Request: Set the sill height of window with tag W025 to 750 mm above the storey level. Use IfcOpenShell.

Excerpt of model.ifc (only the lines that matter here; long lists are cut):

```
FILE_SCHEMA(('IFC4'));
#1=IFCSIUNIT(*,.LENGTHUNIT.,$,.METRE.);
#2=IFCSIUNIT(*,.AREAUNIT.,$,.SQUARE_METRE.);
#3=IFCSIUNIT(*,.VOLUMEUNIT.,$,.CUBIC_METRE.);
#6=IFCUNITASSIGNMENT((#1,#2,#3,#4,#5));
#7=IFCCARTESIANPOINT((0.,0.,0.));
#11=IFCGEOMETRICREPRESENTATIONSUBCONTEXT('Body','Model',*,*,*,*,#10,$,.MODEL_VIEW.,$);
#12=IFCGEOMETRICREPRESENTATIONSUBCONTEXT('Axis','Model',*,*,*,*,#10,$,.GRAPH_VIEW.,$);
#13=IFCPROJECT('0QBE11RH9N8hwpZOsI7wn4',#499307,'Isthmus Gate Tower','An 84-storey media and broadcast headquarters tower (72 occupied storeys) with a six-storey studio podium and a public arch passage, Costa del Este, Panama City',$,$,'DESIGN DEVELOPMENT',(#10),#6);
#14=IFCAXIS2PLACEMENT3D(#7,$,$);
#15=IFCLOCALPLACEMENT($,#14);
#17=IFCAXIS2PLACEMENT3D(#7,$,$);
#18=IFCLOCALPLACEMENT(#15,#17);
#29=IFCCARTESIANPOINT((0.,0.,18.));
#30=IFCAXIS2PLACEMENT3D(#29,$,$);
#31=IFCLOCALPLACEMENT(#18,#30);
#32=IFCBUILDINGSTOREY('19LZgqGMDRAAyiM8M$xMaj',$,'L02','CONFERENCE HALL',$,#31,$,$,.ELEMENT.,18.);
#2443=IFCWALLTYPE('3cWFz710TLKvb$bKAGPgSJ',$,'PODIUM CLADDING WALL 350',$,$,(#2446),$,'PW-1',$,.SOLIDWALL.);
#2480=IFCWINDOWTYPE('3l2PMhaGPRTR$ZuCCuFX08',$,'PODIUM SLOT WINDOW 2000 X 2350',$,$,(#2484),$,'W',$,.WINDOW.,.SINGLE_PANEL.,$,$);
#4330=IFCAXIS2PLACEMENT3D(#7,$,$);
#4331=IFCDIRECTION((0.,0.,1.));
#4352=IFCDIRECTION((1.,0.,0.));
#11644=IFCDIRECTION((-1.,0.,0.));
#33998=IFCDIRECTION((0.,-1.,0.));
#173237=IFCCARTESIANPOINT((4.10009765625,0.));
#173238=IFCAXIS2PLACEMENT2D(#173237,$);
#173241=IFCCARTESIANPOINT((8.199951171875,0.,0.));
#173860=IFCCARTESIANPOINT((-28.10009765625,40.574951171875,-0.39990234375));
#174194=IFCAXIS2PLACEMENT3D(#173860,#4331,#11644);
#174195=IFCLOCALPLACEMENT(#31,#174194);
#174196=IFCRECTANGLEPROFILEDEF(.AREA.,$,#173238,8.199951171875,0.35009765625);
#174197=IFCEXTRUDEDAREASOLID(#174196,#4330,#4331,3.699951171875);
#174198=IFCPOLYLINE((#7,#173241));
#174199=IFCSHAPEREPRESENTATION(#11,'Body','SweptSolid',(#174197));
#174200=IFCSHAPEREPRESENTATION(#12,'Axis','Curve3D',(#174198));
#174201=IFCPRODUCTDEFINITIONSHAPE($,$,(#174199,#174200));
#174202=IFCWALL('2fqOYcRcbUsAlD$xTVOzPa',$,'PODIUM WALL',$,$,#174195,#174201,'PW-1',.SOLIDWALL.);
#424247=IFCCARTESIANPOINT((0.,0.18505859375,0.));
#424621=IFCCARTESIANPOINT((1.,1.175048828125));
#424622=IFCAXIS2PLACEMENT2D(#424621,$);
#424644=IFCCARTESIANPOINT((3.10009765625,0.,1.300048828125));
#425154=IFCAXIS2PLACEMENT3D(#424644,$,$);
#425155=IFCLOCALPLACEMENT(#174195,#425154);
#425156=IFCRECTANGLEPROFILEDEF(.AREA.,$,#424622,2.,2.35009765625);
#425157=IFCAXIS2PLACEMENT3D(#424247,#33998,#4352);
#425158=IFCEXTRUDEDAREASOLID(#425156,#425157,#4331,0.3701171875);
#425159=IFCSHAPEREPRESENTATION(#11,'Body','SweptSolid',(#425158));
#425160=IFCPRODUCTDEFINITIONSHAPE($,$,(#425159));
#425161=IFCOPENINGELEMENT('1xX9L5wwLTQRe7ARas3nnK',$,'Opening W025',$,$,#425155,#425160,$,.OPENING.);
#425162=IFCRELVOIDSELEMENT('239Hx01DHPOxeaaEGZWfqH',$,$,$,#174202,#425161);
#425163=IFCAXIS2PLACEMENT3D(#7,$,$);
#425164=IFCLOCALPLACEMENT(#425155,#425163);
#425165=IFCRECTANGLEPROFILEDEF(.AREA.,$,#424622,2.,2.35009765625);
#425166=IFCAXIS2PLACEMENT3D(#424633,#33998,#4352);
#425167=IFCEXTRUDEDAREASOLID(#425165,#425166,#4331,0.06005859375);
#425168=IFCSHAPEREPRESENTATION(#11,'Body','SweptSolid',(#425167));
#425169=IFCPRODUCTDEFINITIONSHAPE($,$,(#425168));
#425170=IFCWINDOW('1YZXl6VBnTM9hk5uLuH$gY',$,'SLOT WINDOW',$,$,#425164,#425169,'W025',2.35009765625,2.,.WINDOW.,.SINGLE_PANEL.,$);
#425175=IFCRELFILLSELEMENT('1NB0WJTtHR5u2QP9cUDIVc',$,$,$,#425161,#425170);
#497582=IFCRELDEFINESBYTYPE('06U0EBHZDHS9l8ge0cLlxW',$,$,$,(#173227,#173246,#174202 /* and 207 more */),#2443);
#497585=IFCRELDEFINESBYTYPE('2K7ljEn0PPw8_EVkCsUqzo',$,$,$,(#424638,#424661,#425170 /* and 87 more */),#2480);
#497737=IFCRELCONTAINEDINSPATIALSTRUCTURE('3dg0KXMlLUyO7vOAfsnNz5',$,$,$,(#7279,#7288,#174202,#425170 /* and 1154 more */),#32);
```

```python
import numpy as np
import ifcopenshell
import ifcopenshell.api.geometry
import ifcopenshell.geom
import ifcopenshell.util.element
import ifcopenshell.util.placement
import ifcopenshell.util.shape
import ifcopenshell.util.unit

model = ifcopenshell.open("model.ifc")
unit_scale = ifcopenshell.util.unit.calculate_unit_scale(model)

window = model.by_guid("1YZXl6VBnTM9hk5uLuH$gY")
opening = window.FillsVoids[0].RelatingOpeningElement
storey = ifcopenshell.util.element.get_container(window, ifc_class="IfcBuildingStorey")
level = ifcopenshell.util.placement.get_local_placement(storey.ObjectPlacement)[2, 3]

# The opening's origin need not be at the sill, so measure its lowest point.
shape = ifcopenshell.geom.create_shape(ifcopenshell.geom.settings(), opening)
bottom = ifcopenshell.util.shape.get_shape_bottom_elevation(shape, shape.geometry) / unit_scale
dz = level + 0.75 / unit_scale - bottom

shift = np.array([0.0, 0.0, dz])
# The window is placed relative to its opening, so it follows when the opening moves.
matrix = ifcopenshell.util.placement.get_local_placement(opening.ObjectPlacement)
matrix[:3, 3] += shift
ifcopenshell.api.geometry.edit_object_placement(
    model, product=opening, matrix=matrix, is_si=False, should_transform_children=True
)

print(f"moved by {dz * unit_scale:+.3f} m")

model.write("model_edited.ifc")
```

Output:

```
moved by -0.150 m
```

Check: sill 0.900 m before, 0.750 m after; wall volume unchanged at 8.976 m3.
